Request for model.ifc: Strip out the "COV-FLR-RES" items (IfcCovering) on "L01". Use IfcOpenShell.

First a look at what the model holds.

```python
import ifcopenshell
import ifcopenshell.util.element

model = ifcopenshell.open("model.ifc")
print(model.schema)
storey = next(s for s in model.by_type("IfcBuildingStorey") if s.Name == "L01")
coverings = [e for e in ifcopenshell.util.element.get_decomposition(storey) if e.is_a("IfcCovering")]
seen = {}
for e in coverings:
    element_type = ifcopenshell.util.element.get_type(e)
    name = element_type.Name if element_type not in (None, e) else None
    seen[name] = seen.get(name, 0) + 1
for name, count in sorted(seen.items(), key=str):
    print(count, "x", name)
```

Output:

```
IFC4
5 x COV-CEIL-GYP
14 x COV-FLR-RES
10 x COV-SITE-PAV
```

```python
import ifcopenshell
import ifcopenshell.api.root
import ifcopenshell.util.element

model = ifcopenshell.open("model.ifc")

storey = next(s for s in model.by_type("IfcBuildingStorey") if s.Name == "L01")
coverings = [e for e in ifcopenshell.util.element.get_decomposition(storey) if e.is_a("IfcCovering")]
targets = [e for e in coverings if (t := ifcopenshell.util.element.get_type(e)) not in (None, e) and t.Name == "COV-FLR-RES"]

for e in targets:
    ifcopenshell.api.root.remove_product(model, product=e)
print(len(targets), "removed")

model.write("model_v2.ifc")
```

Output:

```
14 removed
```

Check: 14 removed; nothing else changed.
